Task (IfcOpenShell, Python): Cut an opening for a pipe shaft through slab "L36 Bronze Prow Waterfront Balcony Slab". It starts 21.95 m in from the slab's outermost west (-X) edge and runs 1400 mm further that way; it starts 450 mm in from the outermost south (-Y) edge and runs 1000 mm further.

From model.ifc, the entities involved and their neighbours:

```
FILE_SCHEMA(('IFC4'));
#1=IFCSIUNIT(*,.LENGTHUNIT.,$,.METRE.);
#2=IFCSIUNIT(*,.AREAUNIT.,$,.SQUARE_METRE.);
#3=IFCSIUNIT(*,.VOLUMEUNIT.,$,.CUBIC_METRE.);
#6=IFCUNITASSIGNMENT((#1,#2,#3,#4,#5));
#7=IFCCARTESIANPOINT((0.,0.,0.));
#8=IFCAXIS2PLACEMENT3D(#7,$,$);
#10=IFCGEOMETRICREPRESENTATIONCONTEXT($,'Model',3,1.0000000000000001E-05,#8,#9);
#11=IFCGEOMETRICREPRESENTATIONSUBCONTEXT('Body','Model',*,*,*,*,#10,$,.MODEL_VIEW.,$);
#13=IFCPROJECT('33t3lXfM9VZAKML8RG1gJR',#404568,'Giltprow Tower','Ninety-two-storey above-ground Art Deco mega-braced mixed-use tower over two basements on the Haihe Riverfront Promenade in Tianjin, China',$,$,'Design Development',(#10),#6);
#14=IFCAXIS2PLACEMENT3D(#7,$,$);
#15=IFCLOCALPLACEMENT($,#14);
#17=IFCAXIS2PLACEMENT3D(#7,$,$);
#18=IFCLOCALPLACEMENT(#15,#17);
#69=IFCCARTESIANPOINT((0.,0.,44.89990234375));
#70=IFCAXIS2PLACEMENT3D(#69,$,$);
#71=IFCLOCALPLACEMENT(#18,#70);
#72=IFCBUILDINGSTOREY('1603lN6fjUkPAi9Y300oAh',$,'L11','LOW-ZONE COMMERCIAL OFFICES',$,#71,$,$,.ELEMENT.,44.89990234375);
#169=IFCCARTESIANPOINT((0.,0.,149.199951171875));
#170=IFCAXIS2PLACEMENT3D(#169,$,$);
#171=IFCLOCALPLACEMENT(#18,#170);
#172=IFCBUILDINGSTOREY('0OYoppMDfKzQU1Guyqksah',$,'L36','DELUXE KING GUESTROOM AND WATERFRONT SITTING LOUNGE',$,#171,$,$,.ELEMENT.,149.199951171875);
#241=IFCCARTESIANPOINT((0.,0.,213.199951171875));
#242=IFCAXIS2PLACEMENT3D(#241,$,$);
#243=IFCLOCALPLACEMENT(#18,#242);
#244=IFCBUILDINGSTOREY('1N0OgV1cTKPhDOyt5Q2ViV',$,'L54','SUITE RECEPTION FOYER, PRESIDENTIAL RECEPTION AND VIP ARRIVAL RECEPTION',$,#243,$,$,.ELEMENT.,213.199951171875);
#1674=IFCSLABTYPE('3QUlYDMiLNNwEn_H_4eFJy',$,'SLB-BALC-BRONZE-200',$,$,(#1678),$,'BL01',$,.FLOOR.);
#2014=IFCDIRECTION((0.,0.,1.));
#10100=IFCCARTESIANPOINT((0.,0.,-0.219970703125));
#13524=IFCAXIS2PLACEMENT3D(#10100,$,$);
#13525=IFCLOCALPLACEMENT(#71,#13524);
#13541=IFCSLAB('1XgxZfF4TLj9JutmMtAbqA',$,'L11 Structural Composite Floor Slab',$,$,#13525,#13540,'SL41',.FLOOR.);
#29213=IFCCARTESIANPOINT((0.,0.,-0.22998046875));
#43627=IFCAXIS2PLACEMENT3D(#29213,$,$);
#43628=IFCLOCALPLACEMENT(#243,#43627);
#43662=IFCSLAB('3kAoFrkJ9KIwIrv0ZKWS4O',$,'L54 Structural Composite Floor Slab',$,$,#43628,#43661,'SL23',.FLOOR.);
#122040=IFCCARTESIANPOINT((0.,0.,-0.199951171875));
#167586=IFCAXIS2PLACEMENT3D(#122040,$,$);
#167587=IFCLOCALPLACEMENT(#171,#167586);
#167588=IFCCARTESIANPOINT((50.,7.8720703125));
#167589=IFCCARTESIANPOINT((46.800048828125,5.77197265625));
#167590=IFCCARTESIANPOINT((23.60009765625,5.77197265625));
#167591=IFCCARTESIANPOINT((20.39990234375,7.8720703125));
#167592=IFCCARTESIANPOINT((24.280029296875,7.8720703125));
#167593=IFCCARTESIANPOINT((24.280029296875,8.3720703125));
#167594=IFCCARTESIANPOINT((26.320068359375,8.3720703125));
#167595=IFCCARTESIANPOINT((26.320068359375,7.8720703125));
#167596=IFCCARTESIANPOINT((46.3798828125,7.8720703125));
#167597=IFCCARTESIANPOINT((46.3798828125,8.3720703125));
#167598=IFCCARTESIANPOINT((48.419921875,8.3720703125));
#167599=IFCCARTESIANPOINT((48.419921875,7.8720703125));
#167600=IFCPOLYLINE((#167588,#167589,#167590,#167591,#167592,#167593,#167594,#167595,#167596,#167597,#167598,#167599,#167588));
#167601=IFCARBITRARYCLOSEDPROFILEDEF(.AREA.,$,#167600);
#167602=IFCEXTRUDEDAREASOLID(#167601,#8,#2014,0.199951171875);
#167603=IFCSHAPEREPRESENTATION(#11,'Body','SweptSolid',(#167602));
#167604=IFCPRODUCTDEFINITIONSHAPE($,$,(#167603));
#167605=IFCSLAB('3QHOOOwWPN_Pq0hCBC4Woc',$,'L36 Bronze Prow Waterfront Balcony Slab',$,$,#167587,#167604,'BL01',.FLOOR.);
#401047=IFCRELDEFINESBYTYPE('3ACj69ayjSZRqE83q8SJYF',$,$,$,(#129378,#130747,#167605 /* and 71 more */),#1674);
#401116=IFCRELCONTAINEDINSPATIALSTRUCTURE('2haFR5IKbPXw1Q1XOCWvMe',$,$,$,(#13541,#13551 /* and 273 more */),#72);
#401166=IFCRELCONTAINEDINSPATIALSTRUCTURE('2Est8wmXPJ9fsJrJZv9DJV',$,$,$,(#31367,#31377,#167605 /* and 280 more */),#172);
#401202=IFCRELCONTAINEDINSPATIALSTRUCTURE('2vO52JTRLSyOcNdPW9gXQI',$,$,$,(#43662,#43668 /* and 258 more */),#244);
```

```python
import numpy as np
import ifcopenshell
import ifcopenshell.api.feature
import ifcopenshell.api.geometry
import ifcopenshell.api.root
import ifcopenshell.geom
import ifcopenshell.util.placement
import ifcopenshell.util.representation
import ifcopenshell.util.shape
import ifcopenshell.util.unit

model = ifcopenshell.open("model.ifc")
unit_scale = ifcopenshell.util.unit.calculate_unit_scale(model)
settings = ifcopenshell.geom.settings()


def volume(element):
    """Net volume in cubic metres, openings subtracted."""
    shape = ifcopenshell.geom.create_shape(settings, element)
    return ifcopenshell.util.shape.get_volume(shape.geometry)


slab = model.by_guid("3QHOOOwWPN_Pq0hCBC4Woc")
before = volume(slab)

# Extent in the slab's own axes, in metres. The edges named are its -X and -Y sides.
slab_shape = ifcopenshell.geom.create_shape(settings, slab)
vertices = ifcopenshell.util.shape.get_vertices(slab_shape.geometry)
x_min, y_min, bottom = vertices.min(axis=0)
top = vertices[:, 2].max()

opening = ifcopenshell.api.root.create_entity(model, ifc_class="IfcOpeningElement", name="Pipe shaft opening", predefined_type="OPENING")
context = ifcopenshell.util.representation.get_context(model, "Model", "Body", "MODEL_VIEW")
width, depth = 1.4, 1
outline = [(0.0, 0.0), (width, 0.0), (width, depth), (0.0, depth), (0.0, 0.0)]
# Overshoot both faces by 50 mm so the cut is clean.
shape = ifcopenshell.api.geometry.add_slab_representation(
    model, context=context, depth=top - bottom + 0.1, polyline=outline
)
ifcopenshell.api.geometry.assign_representation(model, product=opening, representation=shape)

matrix = ifcopenshell.util.placement.get_local_placement(slab.ObjectPlacement)
matrix[:, 3] = matrix @ np.append(np.array([x_min + 21.95, y_min + 0.45, bottom - 0.05]) / unit_scale, 1.0)
ifcopenshell.api.geometry.edit_object_placement(model, product=opening, matrix=matrix, is_si=False)
ifcopenshell.api.feature.add_feature(model, feature=opening, element=slab)

after = volume(slab)

print(f"slab volume {before:.3f} -> {after:.3f} m3")

model.write("model-out.ifc")
```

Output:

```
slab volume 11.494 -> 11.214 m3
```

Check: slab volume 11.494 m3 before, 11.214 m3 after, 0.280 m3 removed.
